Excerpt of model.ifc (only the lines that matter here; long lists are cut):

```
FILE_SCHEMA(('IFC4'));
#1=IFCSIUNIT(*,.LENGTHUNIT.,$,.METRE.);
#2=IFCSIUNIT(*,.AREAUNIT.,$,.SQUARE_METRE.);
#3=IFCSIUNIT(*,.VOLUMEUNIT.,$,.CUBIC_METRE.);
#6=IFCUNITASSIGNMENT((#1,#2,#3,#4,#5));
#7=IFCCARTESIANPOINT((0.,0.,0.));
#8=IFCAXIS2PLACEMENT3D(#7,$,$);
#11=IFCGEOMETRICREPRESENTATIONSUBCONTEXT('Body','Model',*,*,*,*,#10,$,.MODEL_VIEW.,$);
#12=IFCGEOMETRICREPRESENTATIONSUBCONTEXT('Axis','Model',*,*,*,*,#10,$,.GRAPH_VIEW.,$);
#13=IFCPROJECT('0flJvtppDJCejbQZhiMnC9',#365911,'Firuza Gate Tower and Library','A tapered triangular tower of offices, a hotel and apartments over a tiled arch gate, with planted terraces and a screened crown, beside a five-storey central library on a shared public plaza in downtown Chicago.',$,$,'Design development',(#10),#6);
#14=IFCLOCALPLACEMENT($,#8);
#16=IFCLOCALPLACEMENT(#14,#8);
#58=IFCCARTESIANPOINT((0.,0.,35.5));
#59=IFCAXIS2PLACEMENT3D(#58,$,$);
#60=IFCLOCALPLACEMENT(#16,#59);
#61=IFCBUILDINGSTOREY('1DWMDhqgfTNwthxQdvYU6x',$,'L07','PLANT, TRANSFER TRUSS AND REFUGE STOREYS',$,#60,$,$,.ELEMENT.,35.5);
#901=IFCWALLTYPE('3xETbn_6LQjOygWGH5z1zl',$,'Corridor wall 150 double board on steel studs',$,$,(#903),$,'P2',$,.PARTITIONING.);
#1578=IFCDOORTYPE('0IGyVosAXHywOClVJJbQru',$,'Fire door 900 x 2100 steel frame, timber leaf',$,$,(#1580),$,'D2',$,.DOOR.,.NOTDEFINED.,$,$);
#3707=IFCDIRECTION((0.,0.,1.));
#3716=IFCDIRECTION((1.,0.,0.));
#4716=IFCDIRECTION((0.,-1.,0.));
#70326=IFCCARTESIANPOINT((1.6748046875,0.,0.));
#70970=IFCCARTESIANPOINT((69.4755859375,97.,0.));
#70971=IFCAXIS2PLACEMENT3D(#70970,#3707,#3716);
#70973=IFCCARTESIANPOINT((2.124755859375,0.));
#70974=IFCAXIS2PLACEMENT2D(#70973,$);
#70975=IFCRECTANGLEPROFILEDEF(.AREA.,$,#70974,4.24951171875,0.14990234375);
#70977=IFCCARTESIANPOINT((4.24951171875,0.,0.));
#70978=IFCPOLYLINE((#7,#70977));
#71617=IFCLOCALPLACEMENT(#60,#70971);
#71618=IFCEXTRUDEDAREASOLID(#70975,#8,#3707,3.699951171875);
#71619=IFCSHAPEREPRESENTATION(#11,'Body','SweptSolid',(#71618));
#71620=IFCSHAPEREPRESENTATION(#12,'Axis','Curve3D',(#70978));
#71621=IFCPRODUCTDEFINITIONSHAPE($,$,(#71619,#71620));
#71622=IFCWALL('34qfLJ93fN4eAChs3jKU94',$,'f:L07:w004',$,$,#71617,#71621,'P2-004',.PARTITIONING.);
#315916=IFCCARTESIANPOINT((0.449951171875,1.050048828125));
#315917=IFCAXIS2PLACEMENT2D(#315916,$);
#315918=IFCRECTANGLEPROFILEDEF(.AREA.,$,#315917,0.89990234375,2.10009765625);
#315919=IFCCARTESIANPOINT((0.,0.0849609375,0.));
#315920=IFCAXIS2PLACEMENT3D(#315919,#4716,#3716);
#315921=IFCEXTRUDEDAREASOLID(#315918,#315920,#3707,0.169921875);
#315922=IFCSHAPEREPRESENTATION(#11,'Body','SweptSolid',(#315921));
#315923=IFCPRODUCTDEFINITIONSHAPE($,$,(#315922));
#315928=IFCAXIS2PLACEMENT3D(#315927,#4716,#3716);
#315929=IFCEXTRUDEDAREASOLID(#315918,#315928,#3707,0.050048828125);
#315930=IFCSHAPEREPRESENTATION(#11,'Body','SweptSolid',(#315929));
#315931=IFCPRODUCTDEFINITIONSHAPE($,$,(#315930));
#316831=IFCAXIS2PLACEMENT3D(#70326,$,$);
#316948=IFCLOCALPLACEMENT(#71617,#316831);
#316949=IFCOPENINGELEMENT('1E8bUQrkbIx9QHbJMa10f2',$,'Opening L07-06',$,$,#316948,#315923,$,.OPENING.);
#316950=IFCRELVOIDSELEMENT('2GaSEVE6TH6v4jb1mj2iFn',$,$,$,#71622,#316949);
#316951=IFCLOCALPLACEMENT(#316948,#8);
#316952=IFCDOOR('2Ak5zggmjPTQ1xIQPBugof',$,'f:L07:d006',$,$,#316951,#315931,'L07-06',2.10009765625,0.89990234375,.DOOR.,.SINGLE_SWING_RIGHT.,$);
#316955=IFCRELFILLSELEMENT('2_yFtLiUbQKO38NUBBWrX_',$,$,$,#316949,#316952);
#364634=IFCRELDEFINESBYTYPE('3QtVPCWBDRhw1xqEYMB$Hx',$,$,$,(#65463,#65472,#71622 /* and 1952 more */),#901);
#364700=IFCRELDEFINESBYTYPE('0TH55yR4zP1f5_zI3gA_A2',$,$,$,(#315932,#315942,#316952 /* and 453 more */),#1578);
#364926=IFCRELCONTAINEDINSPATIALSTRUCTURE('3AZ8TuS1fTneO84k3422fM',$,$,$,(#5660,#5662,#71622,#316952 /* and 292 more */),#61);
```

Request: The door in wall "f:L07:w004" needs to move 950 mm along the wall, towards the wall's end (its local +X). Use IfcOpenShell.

```python
import ifcopenshell
import ifcopenshell.api.geometry
import ifcopenshell.util.placement
import ifcopenshell.util.unit

model = ifcopenshell.open("model.ifc")
unit_scale = ifcopenshell.util.unit.calculate_unit_scale(model)

door = model.by_guid("2Ak5zggmjPTQ1xIQPBugof")
opening = door.FillsVoids[0].RelatingOpeningElement
wall = opening.VoidsElements[0].RelatingBuildingElement

wall_matrix = ifcopenshell.util.placement.get_local_placement(wall.ObjectPlacement)
shift = wall_matrix[:3, 0] * 0.95 / unit_scale
before = ifcopenshell.util.placement.get_local_placement(door.ObjectPlacement)[:3, 3].copy()

# The door is placed relative to its opening, so it follows when the opening moves.
matrix = ifcopenshell.util.placement.get_local_placement(opening.ObjectPlacement)
matrix[:3, 3] += shift
ifcopenshell.api.geometry.edit_object_placement(
    model, product=opening, matrix=matrix, is_si=False, should_transform_children=True
)

after = ifcopenshell.util.placement.get_local_placement(door.ObjectPlacement)[:3, 3]
print("door moved by", (after - before).round(3) + 0.0)

model.write("model_rev.ifc")
```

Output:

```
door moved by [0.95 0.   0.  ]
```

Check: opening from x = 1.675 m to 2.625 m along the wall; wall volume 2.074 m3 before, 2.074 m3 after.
